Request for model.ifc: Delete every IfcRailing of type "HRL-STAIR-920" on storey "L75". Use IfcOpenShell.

First a look at what the model holds.

```python
import ifcopenshell
import ifcopenshell.util.element

model = ifcopenshell.open("model.ifc")
print(model.schema)
storey = next(s for s in model.by_type("IfcBuildingStorey") if s.Name == "L75")
railings = [e for e in ifcopenshell.util.element.get_decomposition(storey) if e.is_a("IfcRailing")]
seen = {}
for e in railings:
    element_type = ifcopenshell.util.element.get_type(e)
    name = element_type.Name if element_type not in (None, e) else None
    seen[name] = seen.get(name, 0) + 1
for name, count in sorted(seen.items(), key=str):
    print(count, "x", name)
```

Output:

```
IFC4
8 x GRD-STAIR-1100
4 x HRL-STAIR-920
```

```python
import ifcopenshell
import ifcopenshell.api.root
import ifcopenshell.util.element

model = ifcopenshell.open("model.ifc")

storey = next(s for s in model.by_type("IfcBuildingStorey") if s.Name == "L75")
railings = [e for e in ifcopenshell.util.element.get_decomposition(storey) if e.is_a("IfcRailing")]
targets = [e for e in railings if (t := ifcopenshell.util.element.get_type(e)) not in (None, e) and t.Name == "HRL-STAIR-920"]

for e in targets:
    ifcopenshell.api.root.remove_product(model, product=e)
print(len(targets), "removed")

model.write("model_rev.ifc")
```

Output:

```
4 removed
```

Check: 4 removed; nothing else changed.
